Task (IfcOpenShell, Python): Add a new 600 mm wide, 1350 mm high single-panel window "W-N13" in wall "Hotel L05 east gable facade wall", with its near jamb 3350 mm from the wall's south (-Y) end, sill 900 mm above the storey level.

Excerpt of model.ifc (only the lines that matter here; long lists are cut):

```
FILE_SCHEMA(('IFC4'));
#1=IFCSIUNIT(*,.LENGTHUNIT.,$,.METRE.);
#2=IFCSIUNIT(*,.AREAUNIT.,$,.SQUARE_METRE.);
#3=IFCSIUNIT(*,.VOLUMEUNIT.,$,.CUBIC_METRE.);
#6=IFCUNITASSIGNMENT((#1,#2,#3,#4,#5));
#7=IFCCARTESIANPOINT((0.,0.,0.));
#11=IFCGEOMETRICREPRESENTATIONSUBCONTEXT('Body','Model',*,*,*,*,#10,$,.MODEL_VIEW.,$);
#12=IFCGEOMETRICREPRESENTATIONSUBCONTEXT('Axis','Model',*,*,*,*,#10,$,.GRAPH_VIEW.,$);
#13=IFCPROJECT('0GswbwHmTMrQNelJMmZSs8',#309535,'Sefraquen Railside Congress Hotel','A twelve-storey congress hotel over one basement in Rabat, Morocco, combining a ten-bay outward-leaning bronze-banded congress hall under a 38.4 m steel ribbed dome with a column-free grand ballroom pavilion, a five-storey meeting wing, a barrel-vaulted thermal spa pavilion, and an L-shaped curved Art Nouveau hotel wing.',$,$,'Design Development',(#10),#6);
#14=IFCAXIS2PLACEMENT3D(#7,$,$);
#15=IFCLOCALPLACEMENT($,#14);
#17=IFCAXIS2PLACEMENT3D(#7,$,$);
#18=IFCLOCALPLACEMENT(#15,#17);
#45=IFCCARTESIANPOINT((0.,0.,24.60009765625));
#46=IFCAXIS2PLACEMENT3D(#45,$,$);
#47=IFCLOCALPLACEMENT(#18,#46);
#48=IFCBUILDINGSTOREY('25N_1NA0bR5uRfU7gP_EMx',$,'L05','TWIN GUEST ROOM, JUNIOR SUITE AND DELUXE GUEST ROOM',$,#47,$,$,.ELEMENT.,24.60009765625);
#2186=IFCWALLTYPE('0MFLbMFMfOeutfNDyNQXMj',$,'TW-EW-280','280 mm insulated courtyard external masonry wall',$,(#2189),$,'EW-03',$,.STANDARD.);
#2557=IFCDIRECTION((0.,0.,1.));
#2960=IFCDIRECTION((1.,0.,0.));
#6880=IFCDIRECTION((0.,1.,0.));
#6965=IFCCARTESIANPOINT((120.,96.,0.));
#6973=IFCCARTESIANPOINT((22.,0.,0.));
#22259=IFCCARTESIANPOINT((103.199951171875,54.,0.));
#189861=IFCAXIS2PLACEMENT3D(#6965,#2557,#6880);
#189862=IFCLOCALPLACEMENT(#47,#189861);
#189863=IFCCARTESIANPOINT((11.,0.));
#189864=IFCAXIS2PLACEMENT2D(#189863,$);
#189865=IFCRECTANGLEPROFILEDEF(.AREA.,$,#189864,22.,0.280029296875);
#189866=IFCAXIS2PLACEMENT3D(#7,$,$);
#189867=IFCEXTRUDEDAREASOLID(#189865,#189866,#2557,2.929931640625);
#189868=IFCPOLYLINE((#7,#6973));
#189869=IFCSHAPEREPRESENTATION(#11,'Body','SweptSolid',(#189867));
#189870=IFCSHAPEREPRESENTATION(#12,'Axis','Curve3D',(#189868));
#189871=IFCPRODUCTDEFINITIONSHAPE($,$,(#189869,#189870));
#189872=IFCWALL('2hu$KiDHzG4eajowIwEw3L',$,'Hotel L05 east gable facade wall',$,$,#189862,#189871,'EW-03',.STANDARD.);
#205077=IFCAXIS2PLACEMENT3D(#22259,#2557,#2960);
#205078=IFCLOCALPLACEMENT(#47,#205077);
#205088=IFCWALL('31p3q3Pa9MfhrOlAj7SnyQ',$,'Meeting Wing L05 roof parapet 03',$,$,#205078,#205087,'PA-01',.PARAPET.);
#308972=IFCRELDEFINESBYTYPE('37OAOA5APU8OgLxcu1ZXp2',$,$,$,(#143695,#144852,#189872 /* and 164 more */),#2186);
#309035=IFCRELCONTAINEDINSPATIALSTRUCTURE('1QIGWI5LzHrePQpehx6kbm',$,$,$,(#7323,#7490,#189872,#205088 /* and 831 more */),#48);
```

```python
import numpy as np
import ifcopenshell
import ifcopenshell.api.feature
import ifcopenshell.api.geometry
import ifcopenshell.api.root
import ifcopenshell.api.spatial
import ifcopenshell.geom
import ifcopenshell.util.element
import ifcopenshell.util.placement
import ifcopenshell.util.representation
import ifcopenshell.util.shape
import ifcopenshell.util.unit

model = ifcopenshell.open("model.ifc")
unit_scale = ifcopenshell.util.unit.calculate_unit_scale(model)
settings = ifcopenshell.geom.settings()


def volume(element):
    """Net volume in cubic metres, openings subtracted."""
    shape = ifcopenshell.geom.create_shape(settings, element)
    return ifcopenshell.util.shape.get_volume(shape.geometry)


wall = model.by_guid("2hu$KiDHzG4eajowIwEw3L")
storey = ifcopenshell.util.element.get_container(wall, ifc_class="IfcBuildingStorey")
context = ifcopenshell.util.representation.get_context(model, "Model", "Body", "MODEL_VIEW")
before = volume(wall)

width, height, from_end, sill = 0.6, 1.35, 3.35, 0.9  # metres

# The wall runs along its own X axis, and the end named is its -X end.
wall_shape = ifcopenshell.geom.create_shape(settings, wall)
x, y, z = ifcopenshell.util.shape.get_vertices(wall_shape.geometry).T
start = x.min() + from_end
face, thickness = float(y.min()), float(y.max() - y.min())
wall_matrix = ifcopenshell.util.placement.get_local_placement(wall.ObjectPlacement)
level = ifcopenshell.util.placement.get_local_placement(storey.ObjectPlacement)[2, 3]


def in_wall(x, y):
    """Placement at x, y metres in the wall's axes, at sill height."""
    matrix = wall_matrix.copy()
    matrix[:, 3] = wall_matrix @ np.array([x / unit_scale, y / unit_scale, 0.0, 1.0])
    matrix[2, 3] = level + sill / unit_scale
    return matrix


# Opening: a box that overshoots both wall faces by 50 mm.
opening = ifcopenshell.api.root.create_entity(model, ifc_class="IfcOpeningElement", predefined_type="OPENING")
box = ifcopenshell.api.geometry.add_wall_representation(
    model, context=context, length=width, height=height, thickness=thickness + 0.1
)
ifcopenshell.api.geometry.assign_representation(model, product=opening, representation=box)
ifcopenshell.api.geometry.edit_object_placement(model, product=opening, matrix=in_wall(start, face - 0.05), is_si=False)
ifcopenshell.api.feature.add_feature(model, feature=opening, element=wall)

window = ifcopenshell.api.root.create_entity(model, ifc_class="IfcWindow", name="W-N13", predefined_type="WINDOW")
window.OverallWidth, window.OverallHeight = width / unit_scale, height / unit_scale
window.PartitioningType = "SINGLE_PANEL"
body = ifcopenshell.api.geometry.add_window_representation(
    model,
    context=context,
    overall_width=window.OverallWidth,
    overall_height=window.OverallHeight,
    partition_type="SINGLE_PANEL",
)
ifcopenshell.api.geometry.assign_representation(model, product=window, representation=body)
ifcopenshell.api.spatial.assign_container(model, products=[window], relating_structure=storey)
ifcopenshell.api.feature.add_filling(model, opening=opening, element=window)

# Centre the window in the wall's thickness.
ifcopenshell.api.geometry.edit_object_placement(model, product=window, matrix=in_wall(start, face), is_si=False)
window_shape = ifcopenshell.geom.create_shape(settings, window)
depth = ifcopenshell.util.shape.get_vertices(window_shape.geometry)[:, 1]
offset = face + thickness / 2 - (depth.min() + depth.max()) / 2
ifcopenshell.api.geometry.edit_object_placement(model, product=window, matrix=in_wall(start, offset), is_si=False)

after = volume(wall)

print(f"wall volume {before:.3f} -> {after:.3f} m3")

model.write("model_updated.ifc")
```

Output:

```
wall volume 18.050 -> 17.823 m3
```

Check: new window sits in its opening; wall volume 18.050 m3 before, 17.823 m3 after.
